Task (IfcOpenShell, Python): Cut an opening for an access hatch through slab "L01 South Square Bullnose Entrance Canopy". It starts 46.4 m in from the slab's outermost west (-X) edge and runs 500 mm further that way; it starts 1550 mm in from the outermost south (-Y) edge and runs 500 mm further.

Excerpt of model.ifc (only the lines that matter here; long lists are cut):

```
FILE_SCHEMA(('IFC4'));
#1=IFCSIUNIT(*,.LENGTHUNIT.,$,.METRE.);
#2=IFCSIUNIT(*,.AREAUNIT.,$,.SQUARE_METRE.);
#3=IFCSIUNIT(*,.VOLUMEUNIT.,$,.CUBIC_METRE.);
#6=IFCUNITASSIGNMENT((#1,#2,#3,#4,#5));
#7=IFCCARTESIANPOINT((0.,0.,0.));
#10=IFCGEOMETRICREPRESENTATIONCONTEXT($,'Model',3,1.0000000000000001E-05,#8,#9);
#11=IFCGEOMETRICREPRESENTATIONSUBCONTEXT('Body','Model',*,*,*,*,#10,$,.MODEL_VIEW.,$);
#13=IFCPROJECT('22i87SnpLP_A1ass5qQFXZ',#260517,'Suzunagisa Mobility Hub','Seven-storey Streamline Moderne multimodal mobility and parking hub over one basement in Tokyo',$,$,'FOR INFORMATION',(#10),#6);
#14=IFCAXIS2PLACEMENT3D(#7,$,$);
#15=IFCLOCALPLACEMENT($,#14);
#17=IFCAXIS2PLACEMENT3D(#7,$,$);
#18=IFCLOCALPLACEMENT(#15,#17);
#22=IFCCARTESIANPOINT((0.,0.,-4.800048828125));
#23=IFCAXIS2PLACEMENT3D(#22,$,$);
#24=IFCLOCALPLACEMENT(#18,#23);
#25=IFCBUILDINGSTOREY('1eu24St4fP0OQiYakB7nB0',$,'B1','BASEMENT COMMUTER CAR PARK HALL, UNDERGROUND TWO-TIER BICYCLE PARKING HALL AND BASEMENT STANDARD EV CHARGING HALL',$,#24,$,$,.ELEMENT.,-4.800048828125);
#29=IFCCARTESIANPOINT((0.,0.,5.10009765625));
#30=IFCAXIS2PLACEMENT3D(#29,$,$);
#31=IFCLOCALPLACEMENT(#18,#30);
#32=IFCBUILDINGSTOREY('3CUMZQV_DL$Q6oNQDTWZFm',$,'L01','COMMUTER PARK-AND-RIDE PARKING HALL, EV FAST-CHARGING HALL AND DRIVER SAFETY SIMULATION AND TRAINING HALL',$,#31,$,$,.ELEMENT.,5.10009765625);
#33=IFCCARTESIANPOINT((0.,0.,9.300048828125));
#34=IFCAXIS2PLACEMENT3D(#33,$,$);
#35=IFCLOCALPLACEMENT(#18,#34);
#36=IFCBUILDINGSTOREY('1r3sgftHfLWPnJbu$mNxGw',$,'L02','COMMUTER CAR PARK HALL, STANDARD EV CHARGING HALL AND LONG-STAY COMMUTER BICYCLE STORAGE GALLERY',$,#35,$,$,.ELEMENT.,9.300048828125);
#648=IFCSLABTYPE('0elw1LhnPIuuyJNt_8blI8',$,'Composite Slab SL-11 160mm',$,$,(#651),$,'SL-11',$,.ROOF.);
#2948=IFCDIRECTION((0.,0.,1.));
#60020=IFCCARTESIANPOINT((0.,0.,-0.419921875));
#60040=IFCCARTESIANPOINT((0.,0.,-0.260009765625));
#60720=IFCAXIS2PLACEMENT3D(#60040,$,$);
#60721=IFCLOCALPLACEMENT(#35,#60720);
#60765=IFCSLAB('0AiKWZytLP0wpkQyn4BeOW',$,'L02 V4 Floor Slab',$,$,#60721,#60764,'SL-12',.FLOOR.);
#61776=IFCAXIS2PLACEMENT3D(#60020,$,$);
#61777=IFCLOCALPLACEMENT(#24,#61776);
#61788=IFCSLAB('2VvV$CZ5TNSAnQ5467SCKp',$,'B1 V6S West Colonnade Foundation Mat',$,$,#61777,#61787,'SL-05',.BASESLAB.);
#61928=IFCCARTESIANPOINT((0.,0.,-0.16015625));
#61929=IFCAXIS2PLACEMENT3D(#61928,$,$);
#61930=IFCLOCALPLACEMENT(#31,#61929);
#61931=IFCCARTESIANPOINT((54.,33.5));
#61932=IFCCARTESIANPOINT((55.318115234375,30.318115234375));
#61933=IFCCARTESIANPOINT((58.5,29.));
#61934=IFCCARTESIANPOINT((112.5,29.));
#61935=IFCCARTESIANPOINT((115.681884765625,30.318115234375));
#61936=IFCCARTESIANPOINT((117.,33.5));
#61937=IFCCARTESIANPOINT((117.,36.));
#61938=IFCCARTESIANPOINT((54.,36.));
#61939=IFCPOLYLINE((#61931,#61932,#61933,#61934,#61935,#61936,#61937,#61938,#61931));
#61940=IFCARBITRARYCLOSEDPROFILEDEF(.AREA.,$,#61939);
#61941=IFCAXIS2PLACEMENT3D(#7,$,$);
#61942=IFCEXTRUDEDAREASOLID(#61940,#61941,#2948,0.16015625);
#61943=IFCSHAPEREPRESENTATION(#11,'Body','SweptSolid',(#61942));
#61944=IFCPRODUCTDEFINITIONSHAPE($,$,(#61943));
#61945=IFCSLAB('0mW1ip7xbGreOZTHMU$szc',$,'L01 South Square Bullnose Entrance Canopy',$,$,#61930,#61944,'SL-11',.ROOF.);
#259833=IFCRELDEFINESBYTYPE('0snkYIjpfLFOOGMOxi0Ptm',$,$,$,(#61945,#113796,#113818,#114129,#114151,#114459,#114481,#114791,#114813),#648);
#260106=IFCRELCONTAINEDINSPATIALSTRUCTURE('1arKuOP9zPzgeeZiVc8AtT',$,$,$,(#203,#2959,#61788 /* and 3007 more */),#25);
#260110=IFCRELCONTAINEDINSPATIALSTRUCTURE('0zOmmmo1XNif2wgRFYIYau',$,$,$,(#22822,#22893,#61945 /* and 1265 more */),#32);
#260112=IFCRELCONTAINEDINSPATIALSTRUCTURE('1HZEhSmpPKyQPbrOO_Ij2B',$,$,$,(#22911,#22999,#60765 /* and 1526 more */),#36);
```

```python
import numpy as np
import ifcopenshell
import ifcopenshell.api.feature
import ifcopenshell.api.geometry
import ifcopenshell.api.root
import ifcopenshell.geom
import ifcopenshell.util.placement
import ifcopenshell.util.representation
import ifcopenshell.util.shape
import ifcopenshell.util.unit

model = ifcopenshell.open("model.ifc")
unit_scale = ifcopenshell.util.unit.calculate_unit_scale(model)
settings = ifcopenshell.geom.settings()


def volume(element):
    """Net volume in cubic metres, openings subtracted."""
    shape = ifcopenshell.geom.create_shape(settings, element)
    return ifcopenshell.util.shape.get_volume(shape.geometry)


slab = model.by_id(61945)
before = volume(slab)

# Extent in the slab's own axes, in metres. The edges named are its -X and -Y sides.
slab_shape = ifcopenshell.geom.create_shape(settings, slab)
vertices = ifcopenshell.util.shape.get_vertices(slab_shape.geometry)
x_min, y_min, bottom = vertices.min(axis=0)
top = vertices[:, 2].max()

opening = ifcopenshell.api.root.create_entity(model, ifc_class="IfcOpeningElement", name="Access hatch opening", predefined_type="OPENING")
context = ifcopenshell.util.representation.get_context(model, "Model", "Body", "MODEL_VIEW")
width, depth = 0.5, 0.5
outline = [(0.0, 0.0), (width, 0.0), (width, depth), (0.0, depth), (0.0, 0.0)]
# Overshoot both faces by 50 mm so the cut is clean.
shape = ifcopenshell.api.geometry.add_slab_representation(
    model, context=context, depth=top - bottom + 0.1, polyline=outline
)
ifcopenshell.api.geometry.assign_representation(model, product=opening, representation=shape)

matrix = ifcopenshell.util.placement.get_local_placement(slab.ObjectPlacement)
matrix[:, 3] = matrix @ np.append(np.array([x_min + 46.4, y_min + 1.55, bottom - 0.05]) / unit_scale, 1.0)
ifcopenshell.api.geometry.edit_object_placement(model, product=opening, matrix=matrix, is_si=False)
ifcopenshell.api.feature.add_feature(model, feature=opening, element=slab)

after = volume(slab)

print(f"slab volume {before:.3f} -> {after:.3f} m3")

model.write("model_v2.ifc")
```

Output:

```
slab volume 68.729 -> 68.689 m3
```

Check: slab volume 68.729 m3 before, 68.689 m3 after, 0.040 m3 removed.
